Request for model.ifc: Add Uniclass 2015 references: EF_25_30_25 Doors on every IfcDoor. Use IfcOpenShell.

First a look at what the model holds.

```python
import ifcopenshell

model = ifcopenshell.open("model.ifc")
print(model.schema)
print("classifications:", [c.Name for c in model.by_type("IfcClassification")])
for ifc_class in ("IfcDoor", "IfcRoof", "IfcStair", "IfcWall", "IfcWindow"):
    print(ifc_class, len(model.by_type(ifc_class)))
```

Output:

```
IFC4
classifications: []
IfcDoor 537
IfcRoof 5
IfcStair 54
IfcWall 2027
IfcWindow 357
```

```python
import ifcopenshell
import ifcopenshell.api.classification

model = ifcopenshell.open("model.ifc")

system = ifcopenshell.api.classification.add_classification(model, classification="Uniclass 2015")

codes = {
    "IfcDoor": ("EF_25_30_25", "Doors"),
}
for ifc_class, (code, name) in codes.items():
    products = model.by_type(ifc_class)
    ifcopenshell.api.classification.add_reference(
        model, products=products, classification=system, identification=code, name=name
    )
    print(code, len(products))

model.write("model_v2.ifc")
```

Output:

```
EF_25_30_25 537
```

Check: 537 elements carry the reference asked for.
